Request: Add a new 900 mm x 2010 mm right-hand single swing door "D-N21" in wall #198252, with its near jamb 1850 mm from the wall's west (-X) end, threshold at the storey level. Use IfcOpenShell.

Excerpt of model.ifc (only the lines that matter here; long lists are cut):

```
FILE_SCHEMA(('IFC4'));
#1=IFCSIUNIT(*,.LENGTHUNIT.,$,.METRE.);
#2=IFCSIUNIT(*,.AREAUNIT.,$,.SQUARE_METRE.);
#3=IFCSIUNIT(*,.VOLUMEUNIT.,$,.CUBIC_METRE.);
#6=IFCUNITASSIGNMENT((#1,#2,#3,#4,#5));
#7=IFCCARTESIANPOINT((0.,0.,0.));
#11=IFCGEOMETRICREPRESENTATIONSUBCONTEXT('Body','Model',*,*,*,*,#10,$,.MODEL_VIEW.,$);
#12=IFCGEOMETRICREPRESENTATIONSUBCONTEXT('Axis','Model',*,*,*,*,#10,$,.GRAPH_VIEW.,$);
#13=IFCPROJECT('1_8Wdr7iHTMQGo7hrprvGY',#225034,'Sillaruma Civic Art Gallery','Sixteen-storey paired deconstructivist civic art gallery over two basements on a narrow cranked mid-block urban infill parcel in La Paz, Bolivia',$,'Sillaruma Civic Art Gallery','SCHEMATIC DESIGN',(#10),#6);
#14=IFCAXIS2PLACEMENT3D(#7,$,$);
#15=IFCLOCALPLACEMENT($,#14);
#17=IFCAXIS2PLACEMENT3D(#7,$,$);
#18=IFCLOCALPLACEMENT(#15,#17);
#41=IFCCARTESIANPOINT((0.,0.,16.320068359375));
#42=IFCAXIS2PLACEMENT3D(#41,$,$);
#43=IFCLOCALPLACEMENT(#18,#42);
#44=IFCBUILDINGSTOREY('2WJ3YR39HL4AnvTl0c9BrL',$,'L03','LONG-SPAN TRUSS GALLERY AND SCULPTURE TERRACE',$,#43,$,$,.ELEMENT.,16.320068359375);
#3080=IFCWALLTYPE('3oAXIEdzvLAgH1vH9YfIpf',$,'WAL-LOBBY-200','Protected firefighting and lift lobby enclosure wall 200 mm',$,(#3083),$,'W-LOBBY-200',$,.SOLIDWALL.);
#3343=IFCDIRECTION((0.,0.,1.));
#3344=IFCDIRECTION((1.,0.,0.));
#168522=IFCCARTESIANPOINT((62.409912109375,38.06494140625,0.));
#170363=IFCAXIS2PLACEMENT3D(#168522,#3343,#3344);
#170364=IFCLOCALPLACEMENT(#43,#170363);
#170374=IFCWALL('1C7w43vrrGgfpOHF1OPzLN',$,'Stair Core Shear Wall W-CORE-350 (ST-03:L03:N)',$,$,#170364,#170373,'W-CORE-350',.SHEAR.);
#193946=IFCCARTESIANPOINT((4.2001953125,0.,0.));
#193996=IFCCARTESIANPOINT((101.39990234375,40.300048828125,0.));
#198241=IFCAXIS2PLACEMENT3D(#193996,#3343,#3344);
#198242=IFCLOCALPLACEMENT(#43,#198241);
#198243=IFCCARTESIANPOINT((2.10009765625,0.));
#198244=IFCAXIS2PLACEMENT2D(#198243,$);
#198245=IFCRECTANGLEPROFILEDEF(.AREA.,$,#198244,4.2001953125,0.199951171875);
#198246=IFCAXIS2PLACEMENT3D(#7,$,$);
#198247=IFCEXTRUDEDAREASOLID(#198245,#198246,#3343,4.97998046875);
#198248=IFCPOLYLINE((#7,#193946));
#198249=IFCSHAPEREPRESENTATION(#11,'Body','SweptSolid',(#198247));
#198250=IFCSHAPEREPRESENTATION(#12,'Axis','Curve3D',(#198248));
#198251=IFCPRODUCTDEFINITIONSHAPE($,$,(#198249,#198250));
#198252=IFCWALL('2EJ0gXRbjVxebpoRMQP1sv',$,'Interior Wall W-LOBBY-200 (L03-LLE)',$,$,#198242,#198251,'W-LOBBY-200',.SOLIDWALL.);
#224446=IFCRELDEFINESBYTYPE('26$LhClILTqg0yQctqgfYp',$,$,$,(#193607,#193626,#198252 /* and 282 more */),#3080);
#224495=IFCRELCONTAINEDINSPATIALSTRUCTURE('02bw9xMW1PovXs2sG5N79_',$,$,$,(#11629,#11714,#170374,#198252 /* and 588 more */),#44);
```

```python
import numpy as np
import ifcopenshell
import ifcopenshell.api.feature
import ifcopenshell.api.geometry
import ifcopenshell.api.root
import ifcopenshell.api.spatial
import ifcopenshell.geom
import ifcopenshell.util.element
import ifcopenshell.util.placement
import ifcopenshell.util.representation
import ifcopenshell.util.shape
import ifcopenshell.util.unit

model = ifcopenshell.open("model.ifc")
unit_scale = ifcopenshell.util.unit.calculate_unit_scale(model)
settings = ifcopenshell.geom.settings()


def volume(element):
    """Net volume in cubic metres, openings subtracted."""
    shape = ifcopenshell.geom.create_shape(settings, element)
    return ifcopenshell.util.shape.get_volume(shape.geometry)


wall = model.by_guid("2EJ0gXRbjVxebpoRMQP1sv")
storey = ifcopenshell.util.element.get_container(wall, ifc_class="IfcBuildingStorey")
context = ifcopenshell.util.representation.get_context(model, "Model", "Body", "MODEL_VIEW")
before = volume(wall)

width, height, from_end, sill = 0.9, 2.01, 1.85, 0.0  # metres

# The wall runs along its own X axis, and the end named is its -X end.
wall_shape = ifcopenshell.geom.create_shape(settings, wall)
x, y, z = ifcopenshell.util.shape.get_vertices(wall_shape.geometry).T
start = x.min() + from_end
face, thickness = float(y.min()), float(y.max() - y.min())
wall_matrix = ifcopenshell.util.placement.get_local_placement(wall.ObjectPlacement)
level = ifcopenshell.util.placement.get_local_placement(storey.ObjectPlacement)[2, 3]


def in_wall(x, y):
    """Placement at x, y metres in the wall's axes, at sill height."""
    matrix = wall_matrix.copy()
    matrix[:, 3] = wall_matrix @ np.array([x / unit_scale, y / unit_scale, 0.0, 1.0])
    matrix[2, 3] = level + sill / unit_scale
    return matrix


# Opening: a box that overshoots both wall faces by 50 mm.
opening = ifcopenshell.api.root.create_entity(model, ifc_class="IfcOpeningElement", predefined_type="OPENING")
box = ifcopenshell.api.geometry.add_wall_representation(
    model, context=context, length=width, height=height, thickness=thickness + 0.1
)
ifcopenshell.api.geometry.assign_representation(model, product=opening, representation=box)
ifcopenshell.api.geometry.edit_object_placement(model, product=opening, matrix=in_wall(start, face - 0.05), is_si=False)
ifcopenshell.api.feature.add_feature(model, feature=opening, element=wall)

door = ifcopenshell.api.root.create_entity(model, ifc_class="IfcDoor", name="D-N21", predefined_type="DOOR")
door.OverallWidth, door.OverallHeight = width / unit_scale, height / unit_scale
door.OperationType = "SINGLE_SWING_RIGHT"
body = ifcopenshell.api.geometry.add_door_representation(
    model,
    context=context,
    overall_width=door.OverallWidth,
    overall_height=door.OverallHeight,
    operation_type="SINGLE_SWING_RIGHT",
    lining_properties={"LiningDepth": thickness / unit_scale, "ThresholdDepth": thickness / unit_scale},
)
ifcopenshell.api.geometry.assign_representation(model, product=door, representation=body)
ifcopenshell.api.spatial.assign_container(model, products=[door], relating_structure=storey)
ifcopenshell.api.feature.add_filling(model, opening=opening, element=door)

# The lining spans the wall, so the door starts at the wall face.
ifcopenshell.api.geometry.edit_object_placement(model, product=door, matrix=in_wall(start, face), is_si=False)

after = volume(wall)

print(f"wall volume {before:.3f} -> {after:.3f} m3")

model.write("model_rev.ifc")
```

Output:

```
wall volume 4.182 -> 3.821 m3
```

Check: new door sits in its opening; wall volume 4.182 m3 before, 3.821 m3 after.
